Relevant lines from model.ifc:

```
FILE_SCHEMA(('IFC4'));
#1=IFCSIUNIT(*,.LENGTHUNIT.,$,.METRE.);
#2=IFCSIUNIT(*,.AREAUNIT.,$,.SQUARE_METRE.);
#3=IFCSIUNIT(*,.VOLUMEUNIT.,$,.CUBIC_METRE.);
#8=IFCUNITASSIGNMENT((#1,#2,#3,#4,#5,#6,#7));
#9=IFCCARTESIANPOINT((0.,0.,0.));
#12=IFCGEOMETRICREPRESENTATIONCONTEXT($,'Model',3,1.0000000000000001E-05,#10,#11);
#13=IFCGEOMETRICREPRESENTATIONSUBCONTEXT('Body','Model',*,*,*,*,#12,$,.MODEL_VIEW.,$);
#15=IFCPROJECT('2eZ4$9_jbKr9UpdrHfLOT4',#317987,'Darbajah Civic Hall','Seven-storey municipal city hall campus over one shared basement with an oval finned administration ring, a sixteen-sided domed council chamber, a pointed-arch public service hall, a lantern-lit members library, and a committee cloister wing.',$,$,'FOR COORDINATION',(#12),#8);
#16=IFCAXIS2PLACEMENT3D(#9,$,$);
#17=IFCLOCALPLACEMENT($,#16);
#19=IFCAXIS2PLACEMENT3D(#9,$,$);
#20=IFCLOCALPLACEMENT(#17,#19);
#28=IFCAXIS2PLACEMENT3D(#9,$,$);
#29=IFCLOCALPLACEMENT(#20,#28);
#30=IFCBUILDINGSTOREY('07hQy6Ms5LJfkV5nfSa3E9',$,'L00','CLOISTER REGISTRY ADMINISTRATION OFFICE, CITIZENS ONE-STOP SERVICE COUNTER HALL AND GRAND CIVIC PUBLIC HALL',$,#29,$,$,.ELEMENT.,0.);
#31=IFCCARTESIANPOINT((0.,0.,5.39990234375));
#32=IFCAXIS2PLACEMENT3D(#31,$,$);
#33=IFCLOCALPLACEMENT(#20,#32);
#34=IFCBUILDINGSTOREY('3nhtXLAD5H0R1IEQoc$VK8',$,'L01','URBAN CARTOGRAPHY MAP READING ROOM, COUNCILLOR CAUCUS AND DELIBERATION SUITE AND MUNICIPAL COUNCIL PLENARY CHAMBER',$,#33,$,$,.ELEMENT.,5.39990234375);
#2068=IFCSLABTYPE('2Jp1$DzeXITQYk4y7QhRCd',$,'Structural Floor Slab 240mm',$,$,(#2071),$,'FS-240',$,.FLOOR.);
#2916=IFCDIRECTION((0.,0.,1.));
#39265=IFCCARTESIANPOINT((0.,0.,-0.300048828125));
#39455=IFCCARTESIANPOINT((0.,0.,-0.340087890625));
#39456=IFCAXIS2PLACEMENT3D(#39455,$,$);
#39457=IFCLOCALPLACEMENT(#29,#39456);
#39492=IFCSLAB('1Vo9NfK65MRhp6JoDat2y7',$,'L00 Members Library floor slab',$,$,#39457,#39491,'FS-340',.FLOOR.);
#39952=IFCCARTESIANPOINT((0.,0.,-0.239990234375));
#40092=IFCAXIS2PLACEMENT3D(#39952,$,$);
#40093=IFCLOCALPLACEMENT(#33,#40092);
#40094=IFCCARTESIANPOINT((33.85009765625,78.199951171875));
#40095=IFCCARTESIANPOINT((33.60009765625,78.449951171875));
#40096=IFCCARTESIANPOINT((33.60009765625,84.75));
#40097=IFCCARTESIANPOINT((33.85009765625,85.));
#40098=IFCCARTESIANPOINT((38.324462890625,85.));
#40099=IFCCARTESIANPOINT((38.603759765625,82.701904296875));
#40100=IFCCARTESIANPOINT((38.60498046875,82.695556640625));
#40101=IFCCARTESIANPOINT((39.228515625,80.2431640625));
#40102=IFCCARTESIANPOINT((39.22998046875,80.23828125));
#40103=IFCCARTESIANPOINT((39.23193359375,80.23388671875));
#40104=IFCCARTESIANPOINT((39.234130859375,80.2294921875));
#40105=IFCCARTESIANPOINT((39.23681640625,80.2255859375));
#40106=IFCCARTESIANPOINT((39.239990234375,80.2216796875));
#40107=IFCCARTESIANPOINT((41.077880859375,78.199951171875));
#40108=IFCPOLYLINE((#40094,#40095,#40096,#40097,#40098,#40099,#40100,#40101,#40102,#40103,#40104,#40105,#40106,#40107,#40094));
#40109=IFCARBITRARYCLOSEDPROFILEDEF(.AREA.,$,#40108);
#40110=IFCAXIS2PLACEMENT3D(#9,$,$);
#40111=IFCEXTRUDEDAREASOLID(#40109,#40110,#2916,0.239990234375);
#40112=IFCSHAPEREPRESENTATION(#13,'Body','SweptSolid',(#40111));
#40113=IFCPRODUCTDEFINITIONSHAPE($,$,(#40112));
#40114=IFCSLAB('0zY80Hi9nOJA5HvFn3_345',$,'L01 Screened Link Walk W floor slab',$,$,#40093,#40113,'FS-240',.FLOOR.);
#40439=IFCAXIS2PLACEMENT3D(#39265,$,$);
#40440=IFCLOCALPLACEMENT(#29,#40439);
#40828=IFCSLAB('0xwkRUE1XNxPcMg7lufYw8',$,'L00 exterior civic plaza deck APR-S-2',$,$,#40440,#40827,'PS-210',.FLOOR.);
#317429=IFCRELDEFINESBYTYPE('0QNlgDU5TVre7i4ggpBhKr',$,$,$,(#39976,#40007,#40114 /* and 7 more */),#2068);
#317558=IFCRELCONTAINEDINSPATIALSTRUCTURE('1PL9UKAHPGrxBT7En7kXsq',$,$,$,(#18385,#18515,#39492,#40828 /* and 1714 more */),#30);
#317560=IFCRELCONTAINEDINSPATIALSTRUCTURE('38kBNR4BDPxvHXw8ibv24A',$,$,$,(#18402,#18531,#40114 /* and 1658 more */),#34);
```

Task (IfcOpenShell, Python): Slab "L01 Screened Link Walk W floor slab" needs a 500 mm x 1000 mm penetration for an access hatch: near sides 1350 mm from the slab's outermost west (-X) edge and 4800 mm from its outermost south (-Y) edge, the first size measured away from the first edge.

```python
import numpy as np
import ifcopenshell
import ifcopenshell.api.feature
import ifcopenshell.api.geometry
import ifcopenshell.api.root
import ifcopenshell.geom
import ifcopenshell.util.placement
import ifcopenshell.util.representation
import ifcopenshell.util.shape
import ifcopenshell.util.unit

model = ifcopenshell.open("model.ifc")
unit_scale = ifcopenshell.util.unit.calculate_unit_scale(model)
settings = ifcopenshell.geom.settings()


def volume(element):
    """Net volume in cubic metres, openings subtracted."""
    shape = ifcopenshell.geom.create_shape(settings, element)
    return ifcopenshell.util.shape.get_volume(shape.geometry)


slab = model.by_guid("0zY80Hi9nOJA5HvFn3_345")
before = volume(slab)

# Extent in the slab's own axes, in metres. The edges named are its -X and -Y sides.
slab_shape = ifcopenshell.geom.create_shape(settings, slab)
vertices = ifcopenshell.util.shape.get_vertices(slab_shape.geometry)
x_min, y_min, bottom = vertices.min(axis=0)
top = vertices[:, 2].max()

opening = ifcopenshell.api.root.create_entity(model, ifc_class="IfcOpeningElement", name="Access hatch opening", predefined_type="OPENING")
context = ifcopenshell.util.representation.get_context(model, "Model", "Body", "MODEL_VIEW")
width, depth = 0.5, 1
outline = [(0.0, 0.0), (width, 0.0), (width, depth), (0.0, depth), (0.0, 0.0)]
# Overshoot both faces by 50 mm so the cut is clean.
shape = ifcopenshell.api.geometry.add_slab_representation(
    model, context=context, depth=top - bottom + 0.1, polyline=outline
)
ifcopenshell.api.geometry.assign_representation(model, product=opening, representation=shape)

matrix = ifcopenshell.util.placement.get_local_placement(slab.ObjectPlacement)
matrix[:, 3] = matrix @ np.append(np.array([x_min + 1.35, y_min + 4.8, bottom - 0.05]) / unit_scale, 1.0)
ifcopenshell.api.geometry.edit_object_placement(model, product=opening, matrix=matrix, is_si=False)
ifcopenshell.api.feature.add_feature(model, feature=opening, element=slab)

after = volume(slab)

print(f"slab volume {before:.3f} -> {after:.3f} m3")

model.write("model_updated.ifc")
```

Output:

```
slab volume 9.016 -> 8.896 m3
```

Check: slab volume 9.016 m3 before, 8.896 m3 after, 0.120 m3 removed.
